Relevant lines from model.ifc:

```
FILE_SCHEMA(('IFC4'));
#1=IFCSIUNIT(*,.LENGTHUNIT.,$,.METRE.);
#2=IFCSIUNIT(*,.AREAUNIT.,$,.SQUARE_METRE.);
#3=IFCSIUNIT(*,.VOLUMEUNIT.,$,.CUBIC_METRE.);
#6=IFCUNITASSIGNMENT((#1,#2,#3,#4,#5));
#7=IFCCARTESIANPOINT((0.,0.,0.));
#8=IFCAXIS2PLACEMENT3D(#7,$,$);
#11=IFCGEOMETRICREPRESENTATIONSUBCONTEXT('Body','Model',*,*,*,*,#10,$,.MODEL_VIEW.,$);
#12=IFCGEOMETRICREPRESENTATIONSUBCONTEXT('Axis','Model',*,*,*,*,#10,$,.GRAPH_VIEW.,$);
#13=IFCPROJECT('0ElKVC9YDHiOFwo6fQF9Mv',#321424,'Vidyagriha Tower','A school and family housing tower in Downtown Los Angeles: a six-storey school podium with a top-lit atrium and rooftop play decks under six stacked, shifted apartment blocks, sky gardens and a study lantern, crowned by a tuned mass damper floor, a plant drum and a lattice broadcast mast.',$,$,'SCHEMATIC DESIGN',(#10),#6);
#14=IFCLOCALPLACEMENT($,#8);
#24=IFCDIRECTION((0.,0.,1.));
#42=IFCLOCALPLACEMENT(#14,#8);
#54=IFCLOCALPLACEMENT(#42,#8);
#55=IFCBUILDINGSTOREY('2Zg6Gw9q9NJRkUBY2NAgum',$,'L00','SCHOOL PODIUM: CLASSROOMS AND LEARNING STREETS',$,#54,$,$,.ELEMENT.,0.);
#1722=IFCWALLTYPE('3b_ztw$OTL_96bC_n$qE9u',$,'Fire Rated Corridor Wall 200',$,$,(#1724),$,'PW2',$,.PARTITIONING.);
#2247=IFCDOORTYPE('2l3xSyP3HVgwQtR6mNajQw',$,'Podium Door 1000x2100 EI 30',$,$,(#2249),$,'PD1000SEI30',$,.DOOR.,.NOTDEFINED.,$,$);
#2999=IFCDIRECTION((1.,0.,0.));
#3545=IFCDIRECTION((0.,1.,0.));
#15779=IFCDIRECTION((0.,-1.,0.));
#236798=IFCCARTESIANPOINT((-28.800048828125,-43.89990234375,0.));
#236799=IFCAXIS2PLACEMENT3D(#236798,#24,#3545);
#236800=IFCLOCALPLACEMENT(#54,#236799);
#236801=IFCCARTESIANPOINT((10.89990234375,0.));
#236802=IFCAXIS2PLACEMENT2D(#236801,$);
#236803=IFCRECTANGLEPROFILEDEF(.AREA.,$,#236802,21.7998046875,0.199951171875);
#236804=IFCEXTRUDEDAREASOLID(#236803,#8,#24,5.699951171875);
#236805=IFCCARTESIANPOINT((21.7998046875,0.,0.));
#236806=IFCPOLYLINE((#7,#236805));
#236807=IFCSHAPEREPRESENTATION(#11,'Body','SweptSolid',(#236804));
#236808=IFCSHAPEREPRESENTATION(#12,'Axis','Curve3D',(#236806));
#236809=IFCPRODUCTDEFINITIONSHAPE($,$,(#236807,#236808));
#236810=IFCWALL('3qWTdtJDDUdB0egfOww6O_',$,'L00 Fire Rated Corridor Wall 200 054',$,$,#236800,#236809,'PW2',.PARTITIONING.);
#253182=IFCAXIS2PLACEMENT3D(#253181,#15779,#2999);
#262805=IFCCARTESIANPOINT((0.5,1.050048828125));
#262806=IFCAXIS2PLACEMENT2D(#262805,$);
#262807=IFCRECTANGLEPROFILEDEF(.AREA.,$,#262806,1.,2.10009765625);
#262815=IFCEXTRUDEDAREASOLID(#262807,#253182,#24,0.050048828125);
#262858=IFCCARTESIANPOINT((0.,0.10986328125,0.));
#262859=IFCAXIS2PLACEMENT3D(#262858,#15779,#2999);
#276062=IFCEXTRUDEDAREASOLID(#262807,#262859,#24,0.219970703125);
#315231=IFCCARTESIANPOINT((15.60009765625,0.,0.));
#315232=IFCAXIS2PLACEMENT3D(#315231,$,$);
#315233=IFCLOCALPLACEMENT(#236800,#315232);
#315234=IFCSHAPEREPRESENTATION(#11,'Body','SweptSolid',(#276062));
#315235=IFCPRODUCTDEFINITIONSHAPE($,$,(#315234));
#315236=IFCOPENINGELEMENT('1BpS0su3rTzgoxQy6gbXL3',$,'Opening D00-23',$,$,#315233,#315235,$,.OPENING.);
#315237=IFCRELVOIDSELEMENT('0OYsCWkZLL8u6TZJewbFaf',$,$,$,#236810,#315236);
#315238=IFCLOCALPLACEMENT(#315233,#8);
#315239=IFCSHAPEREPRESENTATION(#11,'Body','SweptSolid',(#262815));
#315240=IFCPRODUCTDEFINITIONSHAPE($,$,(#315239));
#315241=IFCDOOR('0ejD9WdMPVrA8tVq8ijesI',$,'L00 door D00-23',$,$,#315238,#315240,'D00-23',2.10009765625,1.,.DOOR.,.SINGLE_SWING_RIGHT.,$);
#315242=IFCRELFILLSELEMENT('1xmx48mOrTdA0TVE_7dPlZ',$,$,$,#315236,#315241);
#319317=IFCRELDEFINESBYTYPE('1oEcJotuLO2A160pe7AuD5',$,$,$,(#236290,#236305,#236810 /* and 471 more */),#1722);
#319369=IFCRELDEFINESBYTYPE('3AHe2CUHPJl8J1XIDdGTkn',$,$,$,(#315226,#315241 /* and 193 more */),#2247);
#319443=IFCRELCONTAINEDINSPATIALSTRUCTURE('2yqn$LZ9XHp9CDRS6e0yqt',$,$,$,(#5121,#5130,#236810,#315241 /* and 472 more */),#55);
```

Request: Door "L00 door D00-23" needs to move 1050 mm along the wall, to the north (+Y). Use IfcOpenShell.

```python
import ifcopenshell
import ifcopenshell.api.geometry
import ifcopenshell.util.placement
import ifcopenshell.util.unit

model = ifcopenshell.open("model.ifc")
unit_scale = ifcopenshell.util.unit.calculate_unit_scale(model)

door = model.by_id(315241)
opening = door.FillsVoids[0].RelatingOpeningElement
wall = opening.VoidsElements[0].RelatingBuildingElement

wall_matrix = ifcopenshell.util.placement.get_local_placement(wall.ObjectPlacement)
shift = wall_matrix[:3, 0] * 1.05 / unit_scale
before = ifcopenshell.util.placement.get_local_placement(door.ObjectPlacement)[:3, 3].copy()

# The door is placed relative to its opening, so it follows when the opening moves.
matrix = ifcopenshell.util.placement.get_local_placement(opening.ObjectPlacement)
matrix[:3, 3] += shift
ifcopenshell.api.geometry.edit_object_placement(
    model, product=opening, matrix=matrix, is_si=False, should_transform_children=True
)

after = ifcopenshell.util.placement.get_local_placement(door.ObjectPlacement)[:3, 3]
print("door moved by", (after - before).round(3) + 0.0)

model.write("model_updated.ifc")
```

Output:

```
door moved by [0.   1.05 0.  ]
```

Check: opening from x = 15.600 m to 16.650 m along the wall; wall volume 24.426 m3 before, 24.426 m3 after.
